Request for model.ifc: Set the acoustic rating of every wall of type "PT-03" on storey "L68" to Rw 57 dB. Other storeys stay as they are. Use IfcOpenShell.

First a look at what the model holds.

```python
import ifcopenshell
import ifcopenshell.util.element

model = ifcopenshell.open("model.ifc")
print(model.schema)
storey = next(s for s in model.by_type("IfcBuildingStorey") if s.Name == "L68")
walls = [e for e in ifcopenshell.util.element.get_decomposition(storey) if e.is_a("IfcWall")]
seen = {}
for e in walls:
    element_type = ifcopenshell.util.element.get_type(e)
    key = (element_type.Name if element_type != e and element_type else None, ifcopenshell.util.element.get_pset(e, "Pset_WallCommon", "AcousticRating"))
    seen[key] = seen.get(key, 0) + 1
for (name, value), count in sorted(seen.items(), key=str):
    print(count, "x", name, "|", value)
```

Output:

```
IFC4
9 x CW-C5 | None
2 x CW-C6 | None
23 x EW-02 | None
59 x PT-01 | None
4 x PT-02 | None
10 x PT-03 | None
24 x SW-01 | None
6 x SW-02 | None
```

```python
import ifcopenshell
import ifcopenshell.api.pset
import ifcopenshell.util.element

model = ifcopenshell.open("model.ifc")

storey = next(s for s in model.by_type("IfcBuildingStorey") if s.Name == "L68")
walls = [e for e in ifcopenshell.util.element.get_decomposition(storey) if e.is_a("IfcWall")]

count = 0
for e in walls:
    element_type = ifcopenshell.util.element.get_type(e)
    if element_type in (None, e) or element_type.Name != "PT-03":
        continue
    found = ifcopenshell.util.element.get_pset(e, "Pset_WallCommon", should_inherit=False)
    if found:
        pset = model.by_id(found["id"])
        if len(ifcopenshell.util.element.get_elements_by_pset(pset)) > 1:
            pset = ifcopenshell.api.pset.unshare_pset(model, products=[e], pset=pset)[0]
    else:
        pset = ifcopenshell.api.pset.add_pset(model, product=e, name="Pset_WallCommon")
    ifcopenshell.api.pset.edit_pset(model, pset=pset, properties={"AcousticRating": "Rw 57 dB"})
    count += 1

print(count, "walls updated")

model.write("model_v2.ifc")
```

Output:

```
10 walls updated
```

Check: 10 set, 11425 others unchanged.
